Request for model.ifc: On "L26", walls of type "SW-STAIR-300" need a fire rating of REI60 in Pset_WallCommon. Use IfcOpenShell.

First a look at what the model holds.

```python
import ifcopenshell
import ifcopenshell.util.element

model = ifcopenshell.open("model.ifc")
print(model.schema)
storey = next(s for s in model.by_type("IfcBuildingStorey") if s.Name == "L26")
walls = [e for e in ifcopenshell.util.element.get_decomposition(storey) if e.is_a("IfcWall")]
seen = {}
for e in walls:
    element_type = ifcopenshell.util.element.get_type(e)
    key = (element_type.Name if element_type != e and element_type else None, ifcopenshell.util.element.get_pset(e, "Pset_WallCommon", "FireRating"))
    seen[key] = seen.get(key, 0) + 1
for (name, value), count in sorted(seen.items(), key=str):
    print(count, "x", name, "|", value)
```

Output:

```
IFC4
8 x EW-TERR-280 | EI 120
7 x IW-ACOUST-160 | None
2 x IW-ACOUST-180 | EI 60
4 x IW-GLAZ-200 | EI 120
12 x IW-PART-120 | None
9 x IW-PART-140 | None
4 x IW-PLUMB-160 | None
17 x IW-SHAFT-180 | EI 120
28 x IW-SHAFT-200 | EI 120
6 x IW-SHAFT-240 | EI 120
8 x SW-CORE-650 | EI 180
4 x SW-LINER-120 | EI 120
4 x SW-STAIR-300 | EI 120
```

```python
import ifcopenshell
import ifcopenshell.api.pset
import ifcopenshell.util.element

model = ifcopenshell.open("model.ifc")

storey = next(s for s in model.by_type("IfcBuildingStorey") if s.Name == "L26")
walls = [e for e in ifcopenshell.util.element.get_decomposition(storey) if e.is_a("IfcWall")]

count = 0
for e in walls:
    element_type = ifcopenshell.util.element.get_type(e)
    if element_type in (None, e) or element_type.Name != "SW-STAIR-300":
        continue
    found = ifcopenshell.util.element.get_pset(e, "Pset_WallCommon", should_inherit=False)
    if found:
        pset = model.by_id(found["id"])
        if len(ifcopenshell.util.element.get_elements_by_pset(pset)) > 1:
            pset = ifcopenshell.api.pset.unshare_pset(model, products=[e], pset=pset)[0]
    else:
        pset = ifcopenshell.api.pset.add_pset(model, product=e, name="Pset_WallCommon")
    ifcopenshell.api.pset.edit_pset(model, pset=pset, properties={"FireRating": "REI60"})
    count += 1

print(count, "walls updated")

model.write("model_edited.ifc")
```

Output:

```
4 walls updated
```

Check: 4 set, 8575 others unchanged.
